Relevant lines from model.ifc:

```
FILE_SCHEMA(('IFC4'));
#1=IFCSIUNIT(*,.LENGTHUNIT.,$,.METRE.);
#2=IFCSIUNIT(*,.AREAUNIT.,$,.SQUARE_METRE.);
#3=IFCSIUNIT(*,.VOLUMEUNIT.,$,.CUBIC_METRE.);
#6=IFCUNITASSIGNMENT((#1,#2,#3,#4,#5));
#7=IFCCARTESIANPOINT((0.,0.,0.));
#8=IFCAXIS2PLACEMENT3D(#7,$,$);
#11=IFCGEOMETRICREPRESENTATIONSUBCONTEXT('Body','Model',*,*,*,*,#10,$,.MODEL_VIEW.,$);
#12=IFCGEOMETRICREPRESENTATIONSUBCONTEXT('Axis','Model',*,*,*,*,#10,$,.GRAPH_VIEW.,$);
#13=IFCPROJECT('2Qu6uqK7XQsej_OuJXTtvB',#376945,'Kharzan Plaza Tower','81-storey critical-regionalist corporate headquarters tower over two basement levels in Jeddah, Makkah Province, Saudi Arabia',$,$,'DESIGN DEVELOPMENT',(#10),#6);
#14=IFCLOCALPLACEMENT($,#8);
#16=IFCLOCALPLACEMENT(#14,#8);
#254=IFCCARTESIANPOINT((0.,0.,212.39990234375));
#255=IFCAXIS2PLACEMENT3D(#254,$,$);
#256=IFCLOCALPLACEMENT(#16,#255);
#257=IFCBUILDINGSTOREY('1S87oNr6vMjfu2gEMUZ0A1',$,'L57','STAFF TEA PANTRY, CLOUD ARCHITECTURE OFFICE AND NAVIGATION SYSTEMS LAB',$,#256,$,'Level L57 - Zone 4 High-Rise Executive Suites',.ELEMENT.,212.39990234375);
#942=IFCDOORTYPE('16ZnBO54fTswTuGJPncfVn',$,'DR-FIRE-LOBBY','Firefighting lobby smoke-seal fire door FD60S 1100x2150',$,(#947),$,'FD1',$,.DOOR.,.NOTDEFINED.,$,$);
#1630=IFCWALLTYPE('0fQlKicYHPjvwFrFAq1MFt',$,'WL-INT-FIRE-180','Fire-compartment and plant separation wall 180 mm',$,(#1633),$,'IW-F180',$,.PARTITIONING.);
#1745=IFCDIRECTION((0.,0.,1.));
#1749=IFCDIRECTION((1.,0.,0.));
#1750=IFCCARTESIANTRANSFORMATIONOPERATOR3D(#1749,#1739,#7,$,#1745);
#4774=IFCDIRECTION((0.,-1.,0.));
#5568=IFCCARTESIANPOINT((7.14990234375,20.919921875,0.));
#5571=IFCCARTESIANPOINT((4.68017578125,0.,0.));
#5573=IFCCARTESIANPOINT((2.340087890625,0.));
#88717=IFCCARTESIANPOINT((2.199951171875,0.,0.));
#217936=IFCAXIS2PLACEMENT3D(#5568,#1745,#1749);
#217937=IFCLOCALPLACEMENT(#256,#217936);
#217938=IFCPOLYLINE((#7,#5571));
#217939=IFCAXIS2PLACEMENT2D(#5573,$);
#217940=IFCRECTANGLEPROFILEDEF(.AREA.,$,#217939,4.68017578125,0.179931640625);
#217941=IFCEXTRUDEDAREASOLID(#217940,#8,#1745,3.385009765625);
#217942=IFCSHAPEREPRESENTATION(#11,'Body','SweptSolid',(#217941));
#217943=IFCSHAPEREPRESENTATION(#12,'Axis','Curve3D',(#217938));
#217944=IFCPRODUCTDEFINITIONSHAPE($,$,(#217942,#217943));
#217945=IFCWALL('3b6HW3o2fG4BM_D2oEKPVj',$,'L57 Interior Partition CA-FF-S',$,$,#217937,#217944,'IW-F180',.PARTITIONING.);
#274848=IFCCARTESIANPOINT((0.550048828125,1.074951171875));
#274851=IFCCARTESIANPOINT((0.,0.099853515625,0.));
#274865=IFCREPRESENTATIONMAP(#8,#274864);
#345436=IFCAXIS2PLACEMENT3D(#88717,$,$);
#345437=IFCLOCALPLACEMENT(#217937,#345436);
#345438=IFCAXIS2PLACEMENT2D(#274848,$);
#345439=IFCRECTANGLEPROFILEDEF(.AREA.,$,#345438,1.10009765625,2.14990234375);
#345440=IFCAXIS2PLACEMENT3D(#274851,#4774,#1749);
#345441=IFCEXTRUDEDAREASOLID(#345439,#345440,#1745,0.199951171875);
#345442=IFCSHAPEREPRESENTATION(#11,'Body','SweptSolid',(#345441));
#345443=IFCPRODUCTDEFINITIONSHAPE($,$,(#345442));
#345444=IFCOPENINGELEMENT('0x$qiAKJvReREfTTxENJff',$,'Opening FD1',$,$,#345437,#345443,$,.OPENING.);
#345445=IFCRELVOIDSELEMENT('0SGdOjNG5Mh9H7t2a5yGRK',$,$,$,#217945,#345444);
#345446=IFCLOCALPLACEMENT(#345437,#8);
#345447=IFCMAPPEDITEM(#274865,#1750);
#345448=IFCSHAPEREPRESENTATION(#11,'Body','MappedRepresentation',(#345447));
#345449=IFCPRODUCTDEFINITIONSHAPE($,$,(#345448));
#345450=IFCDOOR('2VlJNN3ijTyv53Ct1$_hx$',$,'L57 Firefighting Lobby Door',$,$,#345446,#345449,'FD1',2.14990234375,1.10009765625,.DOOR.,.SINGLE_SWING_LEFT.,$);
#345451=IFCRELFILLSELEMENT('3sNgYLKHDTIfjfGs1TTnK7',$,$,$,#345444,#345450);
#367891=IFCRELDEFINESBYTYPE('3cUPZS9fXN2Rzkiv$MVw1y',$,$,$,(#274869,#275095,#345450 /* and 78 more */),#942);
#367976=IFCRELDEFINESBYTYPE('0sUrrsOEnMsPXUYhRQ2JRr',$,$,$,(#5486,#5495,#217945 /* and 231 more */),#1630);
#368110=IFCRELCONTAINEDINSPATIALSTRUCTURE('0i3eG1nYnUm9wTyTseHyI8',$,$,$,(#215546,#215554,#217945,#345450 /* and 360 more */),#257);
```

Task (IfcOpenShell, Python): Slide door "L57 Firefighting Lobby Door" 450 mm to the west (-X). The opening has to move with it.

```python
import ifcopenshell
import ifcopenshell.api.geometry
import ifcopenshell.util.placement
import ifcopenshell.util.unit

model = ifcopenshell.open("model.ifc")
unit_scale = ifcopenshell.util.unit.calculate_unit_scale(model)

door = model.by_id(345450)
opening = door.FillsVoids[0].RelatingOpeningElement
wall = opening.VoidsElements[0].RelatingBuildingElement

wall_matrix = ifcopenshell.util.placement.get_local_placement(wall.ObjectPlacement)
shift = wall_matrix[:3, 0] * -0.45 / unit_scale
before = ifcopenshell.util.placement.get_local_placement(door.ObjectPlacement)[:3, 3].copy()

# The door is placed relative to its opening, so it follows when the opening moves.
matrix = ifcopenshell.util.placement.get_local_placement(opening.ObjectPlacement)
matrix[:3, 3] += shift
ifcopenshell.api.geometry.edit_object_placement(
    model, product=opening, matrix=matrix, is_si=False, should_transform_children=True
)

after = ifcopenshell.util.placement.get_local_placement(door.ObjectPlacement)[:3, 3]
print("door moved by", (after - before).round(3) + 0.0)

model.write("model_v2.ifc")
```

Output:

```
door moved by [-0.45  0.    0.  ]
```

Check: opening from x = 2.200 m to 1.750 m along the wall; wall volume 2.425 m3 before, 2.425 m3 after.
